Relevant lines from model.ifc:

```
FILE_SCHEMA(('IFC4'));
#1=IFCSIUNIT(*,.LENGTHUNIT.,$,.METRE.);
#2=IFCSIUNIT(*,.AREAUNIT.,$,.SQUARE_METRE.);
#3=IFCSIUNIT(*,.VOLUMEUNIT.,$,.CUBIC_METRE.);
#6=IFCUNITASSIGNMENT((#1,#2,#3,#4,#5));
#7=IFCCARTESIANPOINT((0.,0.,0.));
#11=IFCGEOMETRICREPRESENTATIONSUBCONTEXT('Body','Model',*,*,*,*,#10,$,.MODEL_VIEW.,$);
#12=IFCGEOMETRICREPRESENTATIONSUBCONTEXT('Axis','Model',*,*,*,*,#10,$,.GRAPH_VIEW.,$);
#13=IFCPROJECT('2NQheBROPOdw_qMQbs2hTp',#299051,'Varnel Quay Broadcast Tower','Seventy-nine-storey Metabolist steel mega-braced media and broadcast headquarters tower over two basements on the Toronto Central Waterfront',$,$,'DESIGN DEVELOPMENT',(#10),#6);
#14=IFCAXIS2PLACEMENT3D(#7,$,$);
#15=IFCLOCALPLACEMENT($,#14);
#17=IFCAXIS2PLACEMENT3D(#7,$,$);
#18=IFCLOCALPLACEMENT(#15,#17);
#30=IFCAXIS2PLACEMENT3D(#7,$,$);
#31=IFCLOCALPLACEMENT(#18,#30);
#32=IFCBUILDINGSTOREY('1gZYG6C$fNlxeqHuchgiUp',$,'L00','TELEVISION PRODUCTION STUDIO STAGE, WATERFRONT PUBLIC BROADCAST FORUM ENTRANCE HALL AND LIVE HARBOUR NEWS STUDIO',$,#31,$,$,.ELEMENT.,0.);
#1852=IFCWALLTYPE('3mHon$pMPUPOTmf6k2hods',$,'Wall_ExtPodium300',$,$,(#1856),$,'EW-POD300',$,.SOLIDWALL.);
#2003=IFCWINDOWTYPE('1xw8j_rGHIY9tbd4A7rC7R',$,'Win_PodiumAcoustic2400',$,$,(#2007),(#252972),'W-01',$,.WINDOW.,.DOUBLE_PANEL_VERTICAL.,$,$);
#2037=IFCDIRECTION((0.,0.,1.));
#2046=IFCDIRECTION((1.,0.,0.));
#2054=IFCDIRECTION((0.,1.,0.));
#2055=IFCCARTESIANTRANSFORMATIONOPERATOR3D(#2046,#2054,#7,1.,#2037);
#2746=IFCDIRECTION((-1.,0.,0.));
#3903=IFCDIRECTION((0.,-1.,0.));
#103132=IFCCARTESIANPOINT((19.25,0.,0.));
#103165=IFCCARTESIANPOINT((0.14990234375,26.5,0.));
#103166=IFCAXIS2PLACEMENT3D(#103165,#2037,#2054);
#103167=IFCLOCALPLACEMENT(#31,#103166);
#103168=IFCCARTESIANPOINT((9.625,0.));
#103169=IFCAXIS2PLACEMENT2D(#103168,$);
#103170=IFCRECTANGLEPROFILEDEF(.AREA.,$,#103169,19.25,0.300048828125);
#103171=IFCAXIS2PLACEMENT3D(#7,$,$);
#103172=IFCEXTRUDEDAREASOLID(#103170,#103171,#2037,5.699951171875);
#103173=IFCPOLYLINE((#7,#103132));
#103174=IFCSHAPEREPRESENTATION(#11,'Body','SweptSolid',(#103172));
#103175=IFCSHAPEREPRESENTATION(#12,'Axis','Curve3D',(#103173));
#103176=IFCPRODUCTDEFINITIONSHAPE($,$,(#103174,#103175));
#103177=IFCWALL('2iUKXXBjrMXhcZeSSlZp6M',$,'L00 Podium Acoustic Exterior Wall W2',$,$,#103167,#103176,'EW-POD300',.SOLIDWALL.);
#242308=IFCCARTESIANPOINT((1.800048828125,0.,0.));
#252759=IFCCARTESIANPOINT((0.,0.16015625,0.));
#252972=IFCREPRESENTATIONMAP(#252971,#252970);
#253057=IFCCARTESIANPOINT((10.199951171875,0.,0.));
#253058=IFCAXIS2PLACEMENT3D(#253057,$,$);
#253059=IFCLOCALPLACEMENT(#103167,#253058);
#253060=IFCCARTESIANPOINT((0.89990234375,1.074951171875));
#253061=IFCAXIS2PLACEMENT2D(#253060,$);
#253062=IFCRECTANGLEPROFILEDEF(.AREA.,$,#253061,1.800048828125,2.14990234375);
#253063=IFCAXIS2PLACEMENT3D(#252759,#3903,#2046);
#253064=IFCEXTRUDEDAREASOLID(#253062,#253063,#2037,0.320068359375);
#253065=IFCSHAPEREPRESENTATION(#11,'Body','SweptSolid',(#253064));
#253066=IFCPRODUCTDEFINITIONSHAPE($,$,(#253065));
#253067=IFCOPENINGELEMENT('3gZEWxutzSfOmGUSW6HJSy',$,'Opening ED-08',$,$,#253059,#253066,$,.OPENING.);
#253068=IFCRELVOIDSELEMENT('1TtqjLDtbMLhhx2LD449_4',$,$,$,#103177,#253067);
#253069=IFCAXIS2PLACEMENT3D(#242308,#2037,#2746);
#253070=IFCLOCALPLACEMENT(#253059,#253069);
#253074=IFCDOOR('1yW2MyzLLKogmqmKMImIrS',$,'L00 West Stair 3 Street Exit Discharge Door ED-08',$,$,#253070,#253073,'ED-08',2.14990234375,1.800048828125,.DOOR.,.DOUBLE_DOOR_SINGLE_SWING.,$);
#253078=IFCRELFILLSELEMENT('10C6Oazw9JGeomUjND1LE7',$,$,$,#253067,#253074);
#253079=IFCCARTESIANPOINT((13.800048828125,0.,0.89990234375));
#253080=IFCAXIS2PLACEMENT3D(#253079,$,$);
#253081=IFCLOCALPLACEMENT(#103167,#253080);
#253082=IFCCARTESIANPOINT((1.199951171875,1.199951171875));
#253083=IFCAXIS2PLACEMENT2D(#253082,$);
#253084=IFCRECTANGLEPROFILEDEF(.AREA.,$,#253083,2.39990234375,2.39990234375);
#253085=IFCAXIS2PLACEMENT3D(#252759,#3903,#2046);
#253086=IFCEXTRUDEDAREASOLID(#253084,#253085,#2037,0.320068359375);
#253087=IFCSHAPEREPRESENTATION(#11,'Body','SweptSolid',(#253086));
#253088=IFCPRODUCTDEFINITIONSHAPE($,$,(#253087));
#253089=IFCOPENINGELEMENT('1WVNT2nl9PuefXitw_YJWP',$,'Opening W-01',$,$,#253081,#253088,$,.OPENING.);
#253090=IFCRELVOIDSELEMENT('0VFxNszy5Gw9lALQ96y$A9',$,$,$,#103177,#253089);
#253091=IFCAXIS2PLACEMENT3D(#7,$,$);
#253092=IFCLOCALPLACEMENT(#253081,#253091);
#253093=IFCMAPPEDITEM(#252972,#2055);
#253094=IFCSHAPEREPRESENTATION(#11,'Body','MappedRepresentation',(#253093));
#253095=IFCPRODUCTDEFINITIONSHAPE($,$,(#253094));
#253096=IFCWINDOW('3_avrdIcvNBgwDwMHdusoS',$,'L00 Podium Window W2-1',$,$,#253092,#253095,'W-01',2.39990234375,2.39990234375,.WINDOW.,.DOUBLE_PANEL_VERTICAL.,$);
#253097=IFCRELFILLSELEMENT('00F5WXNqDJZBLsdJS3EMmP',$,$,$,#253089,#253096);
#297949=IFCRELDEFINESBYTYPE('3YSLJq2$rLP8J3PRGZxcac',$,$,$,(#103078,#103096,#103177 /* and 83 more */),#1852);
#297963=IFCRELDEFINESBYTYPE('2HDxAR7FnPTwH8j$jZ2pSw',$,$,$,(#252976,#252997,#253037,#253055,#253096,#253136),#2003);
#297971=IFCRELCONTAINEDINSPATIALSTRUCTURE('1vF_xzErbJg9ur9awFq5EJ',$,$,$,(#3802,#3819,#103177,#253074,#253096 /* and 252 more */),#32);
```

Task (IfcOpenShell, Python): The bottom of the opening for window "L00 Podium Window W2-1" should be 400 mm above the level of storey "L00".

```python
import numpy as np
import ifcopenshell
import ifcopenshell.api.geometry
import ifcopenshell.geom
import ifcopenshell.util.element
import ifcopenshell.util.placement
import ifcopenshell.util.shape
import ifcopenshell.util.unit

model = ifcopenshell.open("model.ifc")
unit_scale = ifcopenshell.util.unit.calculate_unit_scale(model)

window = model.by_guid("3_avrdIcvNBgwDwMHdusoS")
opening = window.FillsVoids[0].RelatingOpeningElement
storey = ifcopenshell.util.element.get_container(window, ifc_class="IfcBuildingStorey")
level = ifcopenshell.util.placement.get_local_placement(storey.ObjectPlacement)[2, 3]

# The opening's origin need not be at the sill, so measure its lowest point.
shape = ifcopenshell.geom.create_shape(ifcopenshell.geom.settings(), opening)
bottom = ifcopenshell.util.shape.get_shape_bottom_elevation(shape, shape.geometry) / unit_scale
dz = level + 0.4 / unit_scale - bottom

shift = np.array([0.0, 0.0, dz])
# The window is placed relative to its opening, so it follows when the opening moves.
matrix = ifcopenshell.util.placement.get_local_placement(opening.ObjectPlacement)
matrix[:3, 3] += shift
ifcopenshell.api.geometry.edit_object_placement(
    model, product=opening, matrix=matrix, is_si=False, should_transform_children=True
)

print(f"moved by {dz * unit_scale:+.3f} m")

model.write("model_rev.ifc")
```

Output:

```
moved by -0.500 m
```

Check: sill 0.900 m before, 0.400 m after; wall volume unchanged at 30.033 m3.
